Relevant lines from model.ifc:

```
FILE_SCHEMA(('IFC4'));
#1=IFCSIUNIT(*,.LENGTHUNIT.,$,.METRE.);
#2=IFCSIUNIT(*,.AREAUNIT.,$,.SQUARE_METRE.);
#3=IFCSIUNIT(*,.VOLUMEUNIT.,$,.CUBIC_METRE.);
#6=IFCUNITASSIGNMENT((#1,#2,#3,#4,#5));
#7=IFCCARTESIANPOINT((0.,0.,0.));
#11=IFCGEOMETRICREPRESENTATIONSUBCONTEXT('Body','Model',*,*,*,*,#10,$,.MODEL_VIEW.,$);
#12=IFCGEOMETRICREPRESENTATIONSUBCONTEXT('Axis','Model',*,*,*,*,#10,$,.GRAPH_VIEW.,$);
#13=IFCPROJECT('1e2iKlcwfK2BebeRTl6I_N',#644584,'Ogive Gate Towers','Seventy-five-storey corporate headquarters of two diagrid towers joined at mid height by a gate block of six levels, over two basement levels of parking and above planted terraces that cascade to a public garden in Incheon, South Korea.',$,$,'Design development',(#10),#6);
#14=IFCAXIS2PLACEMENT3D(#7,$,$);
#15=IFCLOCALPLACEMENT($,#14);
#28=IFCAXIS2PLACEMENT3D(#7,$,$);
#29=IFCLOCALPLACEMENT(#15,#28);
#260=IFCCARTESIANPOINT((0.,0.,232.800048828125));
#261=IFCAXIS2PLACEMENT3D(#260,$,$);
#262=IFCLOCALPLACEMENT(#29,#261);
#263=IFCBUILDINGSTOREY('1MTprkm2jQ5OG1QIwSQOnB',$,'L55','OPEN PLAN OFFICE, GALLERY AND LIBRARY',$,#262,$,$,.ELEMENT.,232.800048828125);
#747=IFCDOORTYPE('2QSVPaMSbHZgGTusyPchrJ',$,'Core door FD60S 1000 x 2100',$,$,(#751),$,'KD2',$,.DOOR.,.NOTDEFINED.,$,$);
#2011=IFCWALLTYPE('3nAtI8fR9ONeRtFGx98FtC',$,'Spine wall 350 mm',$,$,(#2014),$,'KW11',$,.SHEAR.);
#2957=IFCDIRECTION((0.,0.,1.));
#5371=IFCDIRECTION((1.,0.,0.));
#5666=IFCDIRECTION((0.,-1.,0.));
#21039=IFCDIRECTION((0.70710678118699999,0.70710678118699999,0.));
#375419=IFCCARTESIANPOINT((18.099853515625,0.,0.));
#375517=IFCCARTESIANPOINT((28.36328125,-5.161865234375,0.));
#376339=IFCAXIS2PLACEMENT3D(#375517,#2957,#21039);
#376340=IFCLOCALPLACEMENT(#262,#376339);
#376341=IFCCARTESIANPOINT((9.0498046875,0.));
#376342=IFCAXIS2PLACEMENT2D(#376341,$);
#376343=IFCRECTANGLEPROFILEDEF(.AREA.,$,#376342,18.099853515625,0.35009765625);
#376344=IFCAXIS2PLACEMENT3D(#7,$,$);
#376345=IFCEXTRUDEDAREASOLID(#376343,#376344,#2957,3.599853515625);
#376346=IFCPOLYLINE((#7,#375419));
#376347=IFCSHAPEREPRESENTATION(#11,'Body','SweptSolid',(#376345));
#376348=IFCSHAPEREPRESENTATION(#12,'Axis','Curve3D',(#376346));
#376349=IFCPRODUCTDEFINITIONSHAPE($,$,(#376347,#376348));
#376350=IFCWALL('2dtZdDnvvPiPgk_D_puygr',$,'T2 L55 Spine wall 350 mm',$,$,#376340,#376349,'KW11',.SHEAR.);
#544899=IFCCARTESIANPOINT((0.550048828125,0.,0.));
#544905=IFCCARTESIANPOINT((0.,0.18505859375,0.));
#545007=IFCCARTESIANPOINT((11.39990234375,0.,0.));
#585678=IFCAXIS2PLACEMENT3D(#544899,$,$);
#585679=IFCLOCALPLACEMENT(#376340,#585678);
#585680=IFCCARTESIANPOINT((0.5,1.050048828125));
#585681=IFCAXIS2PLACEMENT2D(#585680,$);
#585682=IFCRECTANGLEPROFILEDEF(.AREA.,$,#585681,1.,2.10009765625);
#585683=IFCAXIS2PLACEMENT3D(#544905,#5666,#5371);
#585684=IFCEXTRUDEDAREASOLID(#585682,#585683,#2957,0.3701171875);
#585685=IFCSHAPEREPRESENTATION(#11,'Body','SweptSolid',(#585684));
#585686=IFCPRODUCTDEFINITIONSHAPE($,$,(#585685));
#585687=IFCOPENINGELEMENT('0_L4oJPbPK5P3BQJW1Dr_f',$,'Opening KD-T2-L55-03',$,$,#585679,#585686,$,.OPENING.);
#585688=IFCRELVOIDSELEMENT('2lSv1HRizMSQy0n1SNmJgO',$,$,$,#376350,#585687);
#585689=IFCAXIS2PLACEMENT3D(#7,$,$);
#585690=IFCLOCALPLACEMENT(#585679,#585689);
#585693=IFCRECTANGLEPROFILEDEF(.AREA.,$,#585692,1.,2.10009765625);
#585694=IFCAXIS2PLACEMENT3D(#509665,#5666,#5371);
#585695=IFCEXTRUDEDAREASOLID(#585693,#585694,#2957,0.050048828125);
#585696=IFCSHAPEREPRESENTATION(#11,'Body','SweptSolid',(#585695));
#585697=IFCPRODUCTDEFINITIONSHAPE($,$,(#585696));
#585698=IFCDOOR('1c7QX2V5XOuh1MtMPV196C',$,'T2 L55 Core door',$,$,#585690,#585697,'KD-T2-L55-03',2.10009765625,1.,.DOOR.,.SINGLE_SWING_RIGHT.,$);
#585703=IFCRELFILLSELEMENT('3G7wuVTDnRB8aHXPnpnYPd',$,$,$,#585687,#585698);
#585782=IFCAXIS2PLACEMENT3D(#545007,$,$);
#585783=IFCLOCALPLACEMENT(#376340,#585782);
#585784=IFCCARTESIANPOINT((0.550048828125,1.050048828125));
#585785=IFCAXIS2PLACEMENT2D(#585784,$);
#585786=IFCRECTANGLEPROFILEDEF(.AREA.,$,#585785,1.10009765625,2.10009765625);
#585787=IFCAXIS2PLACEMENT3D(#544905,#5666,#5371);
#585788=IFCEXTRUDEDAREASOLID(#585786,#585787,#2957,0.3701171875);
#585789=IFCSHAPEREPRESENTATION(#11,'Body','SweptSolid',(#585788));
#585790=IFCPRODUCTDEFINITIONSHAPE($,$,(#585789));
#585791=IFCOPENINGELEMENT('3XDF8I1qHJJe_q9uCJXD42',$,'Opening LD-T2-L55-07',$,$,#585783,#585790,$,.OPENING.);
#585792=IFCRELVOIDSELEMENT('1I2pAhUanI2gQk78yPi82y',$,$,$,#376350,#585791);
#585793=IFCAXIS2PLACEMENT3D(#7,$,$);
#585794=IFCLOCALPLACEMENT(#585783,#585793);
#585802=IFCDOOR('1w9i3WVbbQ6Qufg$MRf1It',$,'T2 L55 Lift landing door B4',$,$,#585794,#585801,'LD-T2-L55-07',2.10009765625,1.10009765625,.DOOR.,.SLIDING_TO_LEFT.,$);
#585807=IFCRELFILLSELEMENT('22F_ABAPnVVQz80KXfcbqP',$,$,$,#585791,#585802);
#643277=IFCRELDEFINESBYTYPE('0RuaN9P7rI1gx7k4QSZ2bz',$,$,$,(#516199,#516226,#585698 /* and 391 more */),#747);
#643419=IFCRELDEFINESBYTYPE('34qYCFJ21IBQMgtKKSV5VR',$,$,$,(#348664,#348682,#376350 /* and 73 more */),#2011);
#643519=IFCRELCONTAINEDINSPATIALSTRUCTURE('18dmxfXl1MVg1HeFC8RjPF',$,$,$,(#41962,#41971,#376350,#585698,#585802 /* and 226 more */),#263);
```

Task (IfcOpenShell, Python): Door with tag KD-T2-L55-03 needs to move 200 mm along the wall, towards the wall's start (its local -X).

```python
import ifcopenshell
import ifcopenshell.api.geometry
import ifcopenshell.util.placement
import ifcopenshell.util.unit

model = ifcopenshell.open("model.ifc")
unit_scale = ifcopenshell.util.unit.calculate_unit_scale(model)

door = model.by_guid("1c7QX2V5XOuh1MtMPV196C")
opening = door.FillsVoids[0].RelatingOpeningElement
wall = opening.VoidsElements[0].RelatingBuildingElement

wall_matrix = ifcopenshell.util.placement.get_local_placement(wall.ObjectPlacement)
shift = wall_matrix[:3, 0] * -0.2 / unit_scale
before = ifcopenshell.util.placement.get_local_placement(door.ObjectPlacement)[:3, 3].copy()

# The door is placed relative to its opening, so it follows when the opening moves.
matrix = ifcopenshell.util.placement.get_local_placement(opening.ObjectPlacement)
matrix[:3, 3] += shift
ifcopenshell.api.geometry.edit_object_placement(
    model, product=opening, matrix=matrix, is_si=False, should_transform_children=True
)

after = ifcopenshell.util.placement.get_local_placement(door.ObjectPlacement)[:3, 3]
print("door moved by", (after - before).round(3) + 0.0)

model.write("model_rev.ifc")
```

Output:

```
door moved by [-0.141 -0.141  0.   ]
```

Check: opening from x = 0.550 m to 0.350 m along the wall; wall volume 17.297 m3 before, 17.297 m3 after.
